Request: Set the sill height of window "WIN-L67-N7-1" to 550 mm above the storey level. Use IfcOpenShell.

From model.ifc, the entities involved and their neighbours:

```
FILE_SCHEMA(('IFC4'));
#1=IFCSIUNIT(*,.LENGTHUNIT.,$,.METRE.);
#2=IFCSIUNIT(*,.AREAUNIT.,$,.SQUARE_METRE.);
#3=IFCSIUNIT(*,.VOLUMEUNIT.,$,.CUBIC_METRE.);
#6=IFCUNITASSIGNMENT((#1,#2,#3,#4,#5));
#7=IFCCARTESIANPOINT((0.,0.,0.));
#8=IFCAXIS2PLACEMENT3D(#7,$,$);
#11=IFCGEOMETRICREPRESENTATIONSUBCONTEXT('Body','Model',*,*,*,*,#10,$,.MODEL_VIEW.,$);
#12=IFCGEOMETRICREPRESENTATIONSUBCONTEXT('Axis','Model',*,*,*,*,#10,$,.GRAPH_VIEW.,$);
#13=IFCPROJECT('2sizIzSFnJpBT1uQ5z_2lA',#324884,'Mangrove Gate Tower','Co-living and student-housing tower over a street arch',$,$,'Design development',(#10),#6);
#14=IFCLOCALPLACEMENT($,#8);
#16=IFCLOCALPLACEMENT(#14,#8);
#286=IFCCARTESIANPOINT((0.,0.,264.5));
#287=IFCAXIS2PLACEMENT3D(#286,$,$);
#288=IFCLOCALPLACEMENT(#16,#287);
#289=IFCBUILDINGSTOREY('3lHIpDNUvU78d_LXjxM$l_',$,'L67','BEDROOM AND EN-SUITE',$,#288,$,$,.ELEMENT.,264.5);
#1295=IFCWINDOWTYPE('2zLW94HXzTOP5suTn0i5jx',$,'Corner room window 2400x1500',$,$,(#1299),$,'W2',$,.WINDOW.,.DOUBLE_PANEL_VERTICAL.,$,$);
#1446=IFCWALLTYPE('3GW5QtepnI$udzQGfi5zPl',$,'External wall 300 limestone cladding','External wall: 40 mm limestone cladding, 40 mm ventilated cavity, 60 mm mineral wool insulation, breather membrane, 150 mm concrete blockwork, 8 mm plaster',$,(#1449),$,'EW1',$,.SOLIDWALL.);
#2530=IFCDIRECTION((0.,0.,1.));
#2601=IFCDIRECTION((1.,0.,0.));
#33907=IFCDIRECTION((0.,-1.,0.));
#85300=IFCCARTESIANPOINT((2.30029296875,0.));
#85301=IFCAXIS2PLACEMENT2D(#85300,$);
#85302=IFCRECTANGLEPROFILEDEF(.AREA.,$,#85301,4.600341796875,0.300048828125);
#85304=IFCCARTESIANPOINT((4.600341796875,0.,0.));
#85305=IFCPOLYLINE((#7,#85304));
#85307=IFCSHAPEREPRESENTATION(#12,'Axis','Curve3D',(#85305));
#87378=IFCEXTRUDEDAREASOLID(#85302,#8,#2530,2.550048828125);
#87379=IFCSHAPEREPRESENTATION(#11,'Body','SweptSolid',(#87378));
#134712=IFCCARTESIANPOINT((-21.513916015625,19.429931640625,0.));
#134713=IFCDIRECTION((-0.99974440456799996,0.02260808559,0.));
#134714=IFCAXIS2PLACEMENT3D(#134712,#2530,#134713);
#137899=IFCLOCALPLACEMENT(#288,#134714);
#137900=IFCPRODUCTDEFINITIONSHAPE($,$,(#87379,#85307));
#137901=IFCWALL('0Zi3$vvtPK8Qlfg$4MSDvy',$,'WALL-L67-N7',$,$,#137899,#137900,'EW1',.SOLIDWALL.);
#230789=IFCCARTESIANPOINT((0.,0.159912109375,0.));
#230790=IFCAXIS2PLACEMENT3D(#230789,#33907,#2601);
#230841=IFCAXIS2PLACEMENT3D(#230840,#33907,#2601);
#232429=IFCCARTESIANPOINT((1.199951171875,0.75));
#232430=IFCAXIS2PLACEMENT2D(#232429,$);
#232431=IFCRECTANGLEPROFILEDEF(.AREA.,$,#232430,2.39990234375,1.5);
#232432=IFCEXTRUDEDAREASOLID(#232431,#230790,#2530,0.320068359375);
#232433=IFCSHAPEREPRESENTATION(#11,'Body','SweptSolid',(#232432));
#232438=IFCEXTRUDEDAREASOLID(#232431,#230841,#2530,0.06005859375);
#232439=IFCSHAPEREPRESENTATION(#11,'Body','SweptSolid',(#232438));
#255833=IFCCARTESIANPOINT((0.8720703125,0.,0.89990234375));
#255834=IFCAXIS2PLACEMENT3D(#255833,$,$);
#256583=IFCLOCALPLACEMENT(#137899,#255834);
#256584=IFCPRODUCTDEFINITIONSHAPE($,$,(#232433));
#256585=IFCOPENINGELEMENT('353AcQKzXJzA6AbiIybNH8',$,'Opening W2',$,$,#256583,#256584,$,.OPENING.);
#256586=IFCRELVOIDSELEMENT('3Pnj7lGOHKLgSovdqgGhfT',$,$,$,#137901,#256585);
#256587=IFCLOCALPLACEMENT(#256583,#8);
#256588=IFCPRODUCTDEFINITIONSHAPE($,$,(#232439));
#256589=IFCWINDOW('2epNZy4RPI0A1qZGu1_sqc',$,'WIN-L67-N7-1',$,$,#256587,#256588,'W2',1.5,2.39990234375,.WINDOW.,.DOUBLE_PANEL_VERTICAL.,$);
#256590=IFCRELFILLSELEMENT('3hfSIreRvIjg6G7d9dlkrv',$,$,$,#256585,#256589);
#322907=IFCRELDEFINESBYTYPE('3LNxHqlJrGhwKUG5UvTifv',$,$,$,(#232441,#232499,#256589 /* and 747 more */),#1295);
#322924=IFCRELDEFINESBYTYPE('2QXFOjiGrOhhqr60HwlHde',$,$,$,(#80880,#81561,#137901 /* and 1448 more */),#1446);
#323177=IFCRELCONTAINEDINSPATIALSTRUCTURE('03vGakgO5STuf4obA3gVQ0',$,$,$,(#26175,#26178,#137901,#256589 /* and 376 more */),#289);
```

```python
import numpy as np
import ifcopenshell
import ifcopenshell.api.geometry
import ifcopenshell.geom
import ifcopenshell.util.element
import ifcopenshell.util.placement
import ifcopenshell.util.shape
import ifcopenshell.util.unit

model = ifcopenshell.open("model.ifc")
unit_scale = ifcopenshell.util.unit.calculate_unit_scale(model)

window = model.by_guid("2epNZy4RPI0A1qZGu1_sqc")
opening = window.FillsVoids[0].RelatingOpeningElement
storey = ifcopenshell.util.element.get_container(window, ifc_class="IfcBuildingStorey")
level = ifcopenshell.util.placement.get_local_placement(storey.ObjectPlacement)[2, 3]

# The opening's origin need not be at the sill, so measure its lowest point.
shape = ifcopenshell.geom.create_shape(ifcopenshell.geom.settings(), opening)
bottom = ifcopenshell.util.shape.get_shape_bottom_elevation(shape, shape.geometry) / unit_scale
dz = level + 0.55 / unit_scale - bottom

shift = np.array([0.0, 0.0, dz])
# The window is placed relative to its opening, so it follows when the opening moves.
matrix = ifcopenshell.util.placement.get_local_placement(opening.ObjectPlacement)
matrix[:3, 3] += shift
ifcopenshell.api.geometry.edit_object_placement(
    model, product=opening, matrix=matrix, is_si=False, should_transform_children=True
)

print(f"moved by {dz * unit_scale:+.3f} m")

model.write("model_rev.ifc")
```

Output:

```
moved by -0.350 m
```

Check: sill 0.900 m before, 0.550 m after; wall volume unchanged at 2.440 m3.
